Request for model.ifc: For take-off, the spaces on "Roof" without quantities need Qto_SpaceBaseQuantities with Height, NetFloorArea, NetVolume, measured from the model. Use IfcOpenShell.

First a look at what the model holds.

```python
import ifcopenshell
import ifcopenshell.util.element
import ifcopenshell.util.unit

model = ifcopenshell.open("model.ifc")
print(model.schema)
for unit_type in ("LENGTHUNIT", "AREAUNIT", "VOLUMEUNIT"):
    print(unit_type, ifcopenshell.util.unit.calculate_unit_scale(model, unit_type))
storey = next(s for s in model.by_type("IfcBuildingStorey") if s.Name == "Roof")
spaces = [e for e in ifcopenshell.util.element.get_decomposition(storey) if e.is_a("IfcSpace")]
for e in sorted(spaces, key=lambda e: e.id()):
    print(e.id(), e.is_a(), e.Name, list(ifcopenshell.util.element.get_psets(e, qtos_only=True)), sep=" | ")
```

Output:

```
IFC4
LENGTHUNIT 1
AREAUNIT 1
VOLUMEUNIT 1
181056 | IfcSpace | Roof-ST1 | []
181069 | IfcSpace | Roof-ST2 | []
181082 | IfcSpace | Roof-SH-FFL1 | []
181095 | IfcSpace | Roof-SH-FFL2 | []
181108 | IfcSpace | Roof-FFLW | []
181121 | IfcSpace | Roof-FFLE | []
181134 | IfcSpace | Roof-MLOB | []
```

```python
import ifcopenshell
import ifcopenshell.api.pset
import ifcopenshell.geom
import ifcopenshell.util.element
import ifcopenshell.util.shape
import ifcopenshell.util.unit

model = ifcopenshell.open("model.ifc")
unit_scale = ifcopenshell.util.unit.calculate_unit_scale(model)
area_scale = ifcopenshell.util.unit.calculate_unit_scale(model, "AREAUNIT")
volume_scale = ifcopenshell.util.unit.calculate_unit_scale(model, "VOLUMEUNIT")
settings = ifcopenshell.geom.settings()

storey = next(s for s in model.by_type("IfcBuildingStorey") if s.Name == "Roof")
spaces = [e for e in ifcopenshell.util.element.get_decomposition(storey) if e.is_a("IfcSpace")]

for e in sorted(spaces, key=lambda e: e.id()):
    if ifcopenshell.util.element.get_psets(e, qtos_only=True, should_inherit=False):
        continue
    # Geometry comes back in metres, in the element's own axes.
    shape = ifcopenshell.geom.create_shape(settings, e)
    values = {
        "Height": ifcopenshell.util.shape.get_z(shape.geometry) / unit_scale,
        "NetFloorArea": ifcopenshell.util.shape.get_footprint_area(shape.geometry) / area_scale,
        "NetVolume": ifcopenshell.util.shape.get_volume(shape.geometry) / volume_scale,
    }
    qto = ifcopenshell.api.pset.add_qto(model, product=e, name="Qto_SpaceBaseQuantities")
    ifcopenshell.api.pset.edit_qto(model, qto=qto, properties=values)
    print(e.id(), {k: round(v, 3) for k, v in values.items()})

model.write("model_edited.ifc")
```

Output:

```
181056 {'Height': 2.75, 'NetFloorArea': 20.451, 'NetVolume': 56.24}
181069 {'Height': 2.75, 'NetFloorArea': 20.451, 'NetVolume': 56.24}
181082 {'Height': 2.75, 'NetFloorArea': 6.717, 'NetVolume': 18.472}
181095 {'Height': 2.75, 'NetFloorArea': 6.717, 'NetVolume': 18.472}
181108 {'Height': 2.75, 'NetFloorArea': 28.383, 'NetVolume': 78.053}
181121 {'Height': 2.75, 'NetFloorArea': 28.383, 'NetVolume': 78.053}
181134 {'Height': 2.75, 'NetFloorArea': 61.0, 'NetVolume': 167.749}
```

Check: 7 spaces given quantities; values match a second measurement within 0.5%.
